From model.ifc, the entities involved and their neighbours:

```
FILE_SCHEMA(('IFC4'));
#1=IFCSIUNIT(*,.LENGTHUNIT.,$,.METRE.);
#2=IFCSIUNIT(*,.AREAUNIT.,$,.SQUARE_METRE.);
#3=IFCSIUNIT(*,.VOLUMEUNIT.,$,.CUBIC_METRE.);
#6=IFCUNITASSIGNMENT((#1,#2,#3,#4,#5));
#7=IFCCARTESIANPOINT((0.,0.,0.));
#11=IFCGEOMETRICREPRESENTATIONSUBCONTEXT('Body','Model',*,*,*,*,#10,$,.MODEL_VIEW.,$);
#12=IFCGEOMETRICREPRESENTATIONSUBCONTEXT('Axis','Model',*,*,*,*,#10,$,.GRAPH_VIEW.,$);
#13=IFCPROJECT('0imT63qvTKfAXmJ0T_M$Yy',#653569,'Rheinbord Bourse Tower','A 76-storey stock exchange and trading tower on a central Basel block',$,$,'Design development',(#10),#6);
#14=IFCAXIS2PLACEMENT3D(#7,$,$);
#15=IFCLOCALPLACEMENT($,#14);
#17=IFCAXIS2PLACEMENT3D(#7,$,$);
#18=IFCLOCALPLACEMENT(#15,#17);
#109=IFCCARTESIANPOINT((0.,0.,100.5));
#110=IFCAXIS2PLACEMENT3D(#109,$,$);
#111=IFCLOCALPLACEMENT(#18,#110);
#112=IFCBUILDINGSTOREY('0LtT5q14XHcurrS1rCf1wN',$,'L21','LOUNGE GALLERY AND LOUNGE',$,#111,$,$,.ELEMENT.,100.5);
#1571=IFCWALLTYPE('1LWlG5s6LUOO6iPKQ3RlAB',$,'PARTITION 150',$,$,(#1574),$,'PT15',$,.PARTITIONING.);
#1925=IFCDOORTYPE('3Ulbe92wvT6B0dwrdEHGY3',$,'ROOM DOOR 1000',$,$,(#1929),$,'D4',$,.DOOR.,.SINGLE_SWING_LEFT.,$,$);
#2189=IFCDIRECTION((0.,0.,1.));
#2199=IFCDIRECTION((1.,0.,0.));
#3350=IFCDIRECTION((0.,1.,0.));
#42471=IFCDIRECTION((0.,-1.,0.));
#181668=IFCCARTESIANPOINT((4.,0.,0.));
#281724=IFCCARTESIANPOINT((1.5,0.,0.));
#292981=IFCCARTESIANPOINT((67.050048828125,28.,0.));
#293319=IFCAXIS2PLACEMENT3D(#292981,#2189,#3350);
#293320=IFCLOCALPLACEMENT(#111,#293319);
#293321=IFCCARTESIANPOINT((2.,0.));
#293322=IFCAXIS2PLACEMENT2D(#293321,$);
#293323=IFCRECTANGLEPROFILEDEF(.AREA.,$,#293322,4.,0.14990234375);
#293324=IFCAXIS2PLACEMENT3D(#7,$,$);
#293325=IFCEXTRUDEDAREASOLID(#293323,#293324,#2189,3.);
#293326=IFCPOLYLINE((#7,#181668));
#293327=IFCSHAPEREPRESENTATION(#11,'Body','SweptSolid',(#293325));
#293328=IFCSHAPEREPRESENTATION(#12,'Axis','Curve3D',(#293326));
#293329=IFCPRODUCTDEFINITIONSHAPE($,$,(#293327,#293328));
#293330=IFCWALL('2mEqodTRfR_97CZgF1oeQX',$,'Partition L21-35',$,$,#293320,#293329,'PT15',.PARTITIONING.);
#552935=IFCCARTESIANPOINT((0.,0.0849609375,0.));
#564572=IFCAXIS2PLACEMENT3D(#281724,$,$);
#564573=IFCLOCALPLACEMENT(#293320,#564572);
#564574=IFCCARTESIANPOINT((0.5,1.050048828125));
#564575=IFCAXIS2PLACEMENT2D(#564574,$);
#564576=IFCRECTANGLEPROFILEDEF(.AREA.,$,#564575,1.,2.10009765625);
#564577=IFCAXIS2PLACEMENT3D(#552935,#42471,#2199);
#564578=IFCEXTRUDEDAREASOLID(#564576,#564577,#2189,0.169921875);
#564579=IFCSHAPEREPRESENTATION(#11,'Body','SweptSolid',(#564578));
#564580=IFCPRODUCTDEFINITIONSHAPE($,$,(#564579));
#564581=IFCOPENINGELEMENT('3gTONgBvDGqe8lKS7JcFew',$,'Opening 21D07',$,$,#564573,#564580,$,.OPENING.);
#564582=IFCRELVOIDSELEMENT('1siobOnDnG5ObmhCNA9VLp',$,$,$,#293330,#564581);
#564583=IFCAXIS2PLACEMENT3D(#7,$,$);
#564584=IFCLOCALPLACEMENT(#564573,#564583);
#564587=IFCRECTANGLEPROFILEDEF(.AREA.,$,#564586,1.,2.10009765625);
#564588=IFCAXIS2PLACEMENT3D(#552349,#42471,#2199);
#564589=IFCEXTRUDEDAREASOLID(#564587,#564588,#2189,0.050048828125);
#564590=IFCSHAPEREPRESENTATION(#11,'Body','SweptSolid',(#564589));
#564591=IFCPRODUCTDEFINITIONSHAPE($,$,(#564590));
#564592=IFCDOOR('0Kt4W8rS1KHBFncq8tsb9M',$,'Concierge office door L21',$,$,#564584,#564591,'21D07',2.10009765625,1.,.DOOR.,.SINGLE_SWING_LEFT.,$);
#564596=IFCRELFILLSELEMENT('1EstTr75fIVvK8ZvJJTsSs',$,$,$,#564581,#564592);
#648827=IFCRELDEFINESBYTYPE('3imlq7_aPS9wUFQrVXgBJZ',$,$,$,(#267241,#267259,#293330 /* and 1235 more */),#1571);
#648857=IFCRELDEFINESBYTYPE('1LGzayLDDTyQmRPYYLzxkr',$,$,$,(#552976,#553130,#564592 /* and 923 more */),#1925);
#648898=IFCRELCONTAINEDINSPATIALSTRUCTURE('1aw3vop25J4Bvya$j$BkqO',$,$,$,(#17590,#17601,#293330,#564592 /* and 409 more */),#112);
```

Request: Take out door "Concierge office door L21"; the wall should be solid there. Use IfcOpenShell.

```python
import ifcopenshell
import ifcopenshell.api.feature
import ifcopenshell.api.root
import ifcopenshell.geom
import ifcopenshell.util.shape

model = ifcopenshell.open("model.ifc")
settings = ifcopenshell.geom.settings()


def volume(element):
    """Net volume in cubic metres, openings subtracted."""
    shape = ifcopenshell.geom.create_shape(settings, element)
    return ifcopenshell.util.shape.get_volume(shape.geometry)


door = model.by_id(564592)
opening = door.FillsVoids[0].RelatingOpeningElement
wall = opening.VoidsElements[0].RelatingBuildingElement
before = volume(wall)

ifcopenshell.api.root.remove_product(model, product=door)
ifcopenshell.api.feature.remove_feature(model, feature=opening)

after = volume(wall)

print(f"wall volume {before:.3f} -> {after:.3f} m3")

model.write("model-out.ifc")
```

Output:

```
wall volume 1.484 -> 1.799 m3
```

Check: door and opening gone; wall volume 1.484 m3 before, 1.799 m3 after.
